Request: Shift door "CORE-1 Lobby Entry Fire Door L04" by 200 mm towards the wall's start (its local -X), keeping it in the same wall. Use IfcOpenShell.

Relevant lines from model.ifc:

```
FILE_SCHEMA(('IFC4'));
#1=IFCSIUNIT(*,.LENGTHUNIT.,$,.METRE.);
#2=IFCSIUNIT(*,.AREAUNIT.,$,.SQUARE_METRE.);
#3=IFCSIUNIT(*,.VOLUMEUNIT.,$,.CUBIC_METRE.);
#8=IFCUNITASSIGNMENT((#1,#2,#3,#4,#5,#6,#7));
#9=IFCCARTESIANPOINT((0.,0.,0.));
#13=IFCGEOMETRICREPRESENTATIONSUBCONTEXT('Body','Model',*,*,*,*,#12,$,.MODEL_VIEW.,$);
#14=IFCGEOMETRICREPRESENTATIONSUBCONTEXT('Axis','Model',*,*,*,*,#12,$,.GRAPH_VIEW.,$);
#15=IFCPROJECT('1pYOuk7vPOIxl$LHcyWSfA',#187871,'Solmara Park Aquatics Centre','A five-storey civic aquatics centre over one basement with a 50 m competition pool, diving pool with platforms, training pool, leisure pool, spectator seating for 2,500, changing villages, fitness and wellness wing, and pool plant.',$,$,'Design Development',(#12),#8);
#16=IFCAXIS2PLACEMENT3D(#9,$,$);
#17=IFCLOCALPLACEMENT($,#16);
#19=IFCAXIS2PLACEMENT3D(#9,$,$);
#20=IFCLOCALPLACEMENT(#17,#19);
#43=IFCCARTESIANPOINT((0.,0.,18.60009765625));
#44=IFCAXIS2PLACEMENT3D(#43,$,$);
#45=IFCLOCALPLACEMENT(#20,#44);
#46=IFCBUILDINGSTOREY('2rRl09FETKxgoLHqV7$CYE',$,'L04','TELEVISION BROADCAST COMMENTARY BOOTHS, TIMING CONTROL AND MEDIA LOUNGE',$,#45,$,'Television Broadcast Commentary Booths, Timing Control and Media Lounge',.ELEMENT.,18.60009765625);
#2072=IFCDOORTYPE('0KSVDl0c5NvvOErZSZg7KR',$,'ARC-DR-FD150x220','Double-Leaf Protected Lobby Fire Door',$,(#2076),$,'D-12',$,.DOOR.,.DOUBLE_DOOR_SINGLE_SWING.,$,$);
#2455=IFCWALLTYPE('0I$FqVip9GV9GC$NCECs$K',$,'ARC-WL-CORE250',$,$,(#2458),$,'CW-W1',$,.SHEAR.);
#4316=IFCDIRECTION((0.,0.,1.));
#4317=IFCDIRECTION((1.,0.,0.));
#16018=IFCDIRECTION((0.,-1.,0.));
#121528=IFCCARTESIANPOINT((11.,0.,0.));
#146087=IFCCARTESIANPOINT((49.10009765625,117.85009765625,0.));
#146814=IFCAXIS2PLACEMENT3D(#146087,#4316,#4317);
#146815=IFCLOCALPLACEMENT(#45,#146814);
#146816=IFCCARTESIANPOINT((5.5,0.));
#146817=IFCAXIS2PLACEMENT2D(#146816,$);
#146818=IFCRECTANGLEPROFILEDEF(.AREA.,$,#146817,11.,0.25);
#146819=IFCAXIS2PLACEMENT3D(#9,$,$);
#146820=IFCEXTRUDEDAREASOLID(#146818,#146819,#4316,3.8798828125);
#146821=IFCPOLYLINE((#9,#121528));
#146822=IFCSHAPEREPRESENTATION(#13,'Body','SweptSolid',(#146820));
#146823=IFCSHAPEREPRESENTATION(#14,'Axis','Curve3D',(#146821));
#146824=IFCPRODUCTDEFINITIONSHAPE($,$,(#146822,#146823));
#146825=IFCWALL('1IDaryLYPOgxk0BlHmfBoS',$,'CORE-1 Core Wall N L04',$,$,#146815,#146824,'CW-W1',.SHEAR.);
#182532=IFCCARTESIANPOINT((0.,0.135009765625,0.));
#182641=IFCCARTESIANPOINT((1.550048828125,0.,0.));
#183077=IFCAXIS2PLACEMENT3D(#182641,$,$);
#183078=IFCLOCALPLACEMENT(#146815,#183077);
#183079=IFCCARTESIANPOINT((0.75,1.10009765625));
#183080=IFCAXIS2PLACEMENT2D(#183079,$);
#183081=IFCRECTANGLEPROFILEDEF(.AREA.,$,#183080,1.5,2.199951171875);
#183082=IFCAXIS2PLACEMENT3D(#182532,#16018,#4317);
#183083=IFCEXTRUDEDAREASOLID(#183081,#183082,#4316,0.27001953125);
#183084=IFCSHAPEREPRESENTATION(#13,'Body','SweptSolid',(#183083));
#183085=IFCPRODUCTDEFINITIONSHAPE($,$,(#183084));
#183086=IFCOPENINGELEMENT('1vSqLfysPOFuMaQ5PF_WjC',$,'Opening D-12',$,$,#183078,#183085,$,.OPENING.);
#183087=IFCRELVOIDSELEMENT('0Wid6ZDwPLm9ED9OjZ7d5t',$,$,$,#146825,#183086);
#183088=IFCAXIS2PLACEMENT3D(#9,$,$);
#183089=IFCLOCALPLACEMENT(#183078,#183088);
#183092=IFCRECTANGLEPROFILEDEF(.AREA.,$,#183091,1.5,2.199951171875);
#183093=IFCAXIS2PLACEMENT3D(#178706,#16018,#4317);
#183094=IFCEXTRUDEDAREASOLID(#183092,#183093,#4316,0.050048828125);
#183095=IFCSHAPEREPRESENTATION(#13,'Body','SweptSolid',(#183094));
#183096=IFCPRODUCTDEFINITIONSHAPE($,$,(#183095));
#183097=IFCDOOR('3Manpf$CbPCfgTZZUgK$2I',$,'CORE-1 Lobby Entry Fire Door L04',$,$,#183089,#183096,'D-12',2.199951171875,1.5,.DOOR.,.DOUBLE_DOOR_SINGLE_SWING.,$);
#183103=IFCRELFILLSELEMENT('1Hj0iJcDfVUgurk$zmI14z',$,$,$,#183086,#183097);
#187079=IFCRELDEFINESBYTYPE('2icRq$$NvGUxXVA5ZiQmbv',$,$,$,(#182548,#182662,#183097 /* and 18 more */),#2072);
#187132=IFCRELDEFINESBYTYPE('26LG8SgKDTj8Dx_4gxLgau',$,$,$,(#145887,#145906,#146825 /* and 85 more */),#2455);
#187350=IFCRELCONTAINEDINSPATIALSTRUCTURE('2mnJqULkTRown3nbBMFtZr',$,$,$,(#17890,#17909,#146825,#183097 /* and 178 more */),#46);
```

```python
import ifcopenshell
import ifcopenshell.api.geometry
import ifcopenshell.util.placement
import ifcopenshell.util.unit

model = ifcopenshell.open("model.ifc")
unit_scale = ifcopenshell.util.unit.calculate_unit_scale(model)

door = model.by_guid("3Manpf$CbPCfgTZZUgK$2I")
opening = door.FillsVoids[0].RelatingOpeningElement
wall = opening.VoidsElements[0].RelatingBuildingElement

wall_matrix = ifcopenshell.util.placement.get_local_placement(wall.ObjectPlacement)
shift = wall_matrix[:3, 0] * -0.2 / unit_scale
before = ifcopenshell.util.placement.get_local_placement(door.ObjectPlacement)[:3, 3].copy()

# The door is placed relative to its opening, so it follows when the opening moves.
matrix = ifcopenshell.util.placement.get_local_placement(opening.ObjectPlacement)
matrix[:3, 3] += shift
ifcopenshell.api.geometry.edit_object_placement(
    model, product=opening, matrix=matrix, is_si=False, should_transform_children=True
)

after = ifcopenshell.util.placement.get_local_placement(door.ObjectPlacement)[:3, 3]
print("door moved by", (after - before).round(3) + 0.0)

model.write("model-out.ifc")
```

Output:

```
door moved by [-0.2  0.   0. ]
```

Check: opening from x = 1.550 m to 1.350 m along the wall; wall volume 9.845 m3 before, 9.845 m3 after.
